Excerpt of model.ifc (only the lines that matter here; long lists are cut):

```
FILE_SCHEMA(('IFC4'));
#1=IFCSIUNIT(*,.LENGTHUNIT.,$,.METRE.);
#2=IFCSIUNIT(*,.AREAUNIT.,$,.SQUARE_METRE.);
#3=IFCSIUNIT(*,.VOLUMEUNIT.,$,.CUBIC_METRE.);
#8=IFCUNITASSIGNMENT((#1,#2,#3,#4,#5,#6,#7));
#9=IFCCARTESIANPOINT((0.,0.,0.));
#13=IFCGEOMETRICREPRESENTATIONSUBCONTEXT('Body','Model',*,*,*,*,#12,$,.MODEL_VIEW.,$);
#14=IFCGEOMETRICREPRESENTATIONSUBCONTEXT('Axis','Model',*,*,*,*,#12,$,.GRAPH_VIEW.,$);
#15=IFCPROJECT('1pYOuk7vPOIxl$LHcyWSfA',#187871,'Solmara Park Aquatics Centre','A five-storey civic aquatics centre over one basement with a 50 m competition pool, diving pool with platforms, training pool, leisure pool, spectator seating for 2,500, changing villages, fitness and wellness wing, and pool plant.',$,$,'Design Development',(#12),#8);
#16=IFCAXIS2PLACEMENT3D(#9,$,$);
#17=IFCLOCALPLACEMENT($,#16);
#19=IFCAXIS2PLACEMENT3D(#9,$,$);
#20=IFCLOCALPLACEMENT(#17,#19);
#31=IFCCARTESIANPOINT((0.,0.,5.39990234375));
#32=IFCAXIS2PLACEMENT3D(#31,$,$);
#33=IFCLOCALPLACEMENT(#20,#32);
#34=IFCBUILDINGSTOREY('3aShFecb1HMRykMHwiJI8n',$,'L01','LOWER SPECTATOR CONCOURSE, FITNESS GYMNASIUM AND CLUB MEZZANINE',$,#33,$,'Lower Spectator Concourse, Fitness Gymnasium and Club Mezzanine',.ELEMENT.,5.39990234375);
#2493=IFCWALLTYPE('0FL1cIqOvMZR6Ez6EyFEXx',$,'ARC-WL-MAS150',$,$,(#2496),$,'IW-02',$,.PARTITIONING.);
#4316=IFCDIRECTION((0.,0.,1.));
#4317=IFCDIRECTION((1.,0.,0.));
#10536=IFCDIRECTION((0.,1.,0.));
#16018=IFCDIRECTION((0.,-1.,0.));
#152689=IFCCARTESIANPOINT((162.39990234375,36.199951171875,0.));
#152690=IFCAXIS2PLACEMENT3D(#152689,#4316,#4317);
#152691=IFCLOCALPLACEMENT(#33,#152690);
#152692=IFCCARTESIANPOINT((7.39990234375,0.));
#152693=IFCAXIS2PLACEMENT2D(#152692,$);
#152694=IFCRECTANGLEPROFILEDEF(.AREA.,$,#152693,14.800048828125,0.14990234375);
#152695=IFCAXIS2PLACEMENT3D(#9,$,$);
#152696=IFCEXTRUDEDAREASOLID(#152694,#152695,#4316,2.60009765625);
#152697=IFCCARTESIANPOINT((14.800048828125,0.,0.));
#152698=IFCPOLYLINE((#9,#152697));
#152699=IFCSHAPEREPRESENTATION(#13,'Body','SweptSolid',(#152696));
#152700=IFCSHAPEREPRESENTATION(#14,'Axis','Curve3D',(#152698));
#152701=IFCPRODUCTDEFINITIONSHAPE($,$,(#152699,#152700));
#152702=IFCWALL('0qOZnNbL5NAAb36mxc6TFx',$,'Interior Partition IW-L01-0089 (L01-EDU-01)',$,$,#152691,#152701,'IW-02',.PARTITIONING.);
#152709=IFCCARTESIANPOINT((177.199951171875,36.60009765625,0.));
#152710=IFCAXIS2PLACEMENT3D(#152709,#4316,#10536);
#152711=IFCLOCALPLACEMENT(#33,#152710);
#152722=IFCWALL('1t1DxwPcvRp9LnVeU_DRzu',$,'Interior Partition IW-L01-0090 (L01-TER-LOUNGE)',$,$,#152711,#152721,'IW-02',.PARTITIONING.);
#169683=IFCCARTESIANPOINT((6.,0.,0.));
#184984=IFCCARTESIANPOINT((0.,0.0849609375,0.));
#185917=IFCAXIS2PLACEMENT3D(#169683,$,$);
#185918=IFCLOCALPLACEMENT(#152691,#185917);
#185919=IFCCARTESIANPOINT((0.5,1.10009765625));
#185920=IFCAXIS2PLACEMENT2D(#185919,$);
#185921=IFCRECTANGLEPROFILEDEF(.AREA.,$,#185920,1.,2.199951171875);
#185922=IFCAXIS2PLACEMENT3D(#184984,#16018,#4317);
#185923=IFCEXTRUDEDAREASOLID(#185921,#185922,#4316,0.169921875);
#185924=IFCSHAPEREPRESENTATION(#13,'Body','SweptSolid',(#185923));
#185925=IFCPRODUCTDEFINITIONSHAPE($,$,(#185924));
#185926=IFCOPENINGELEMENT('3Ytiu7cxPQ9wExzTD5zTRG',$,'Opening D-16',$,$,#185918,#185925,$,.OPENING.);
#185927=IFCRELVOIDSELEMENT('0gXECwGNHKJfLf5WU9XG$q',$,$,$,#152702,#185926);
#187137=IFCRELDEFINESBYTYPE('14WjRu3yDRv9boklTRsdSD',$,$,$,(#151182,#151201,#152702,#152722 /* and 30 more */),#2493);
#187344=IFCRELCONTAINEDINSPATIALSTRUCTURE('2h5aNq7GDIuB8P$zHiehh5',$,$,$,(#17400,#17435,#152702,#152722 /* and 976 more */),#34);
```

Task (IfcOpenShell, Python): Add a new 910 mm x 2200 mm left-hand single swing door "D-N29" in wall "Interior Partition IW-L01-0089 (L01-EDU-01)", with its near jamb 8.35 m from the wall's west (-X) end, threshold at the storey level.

```python
import numpy as np
import ifcopenshell
import ifcopenshell.api.feature
import ifcopenshell.api.geometry
import ifcopenshell.api.root
import ifcopenshell.api.spatial
import ifcopenshell.geom
import ifcopenshell.util.element
import ifcopenshell.util.placement
import ifcopenshell.util.representation
import ifcopenshell.util.shape
import ifcopenshell.util.unit

model = ifcopenshell.open("model.ifc")
unit_scale = ifcopenshell.util.unit.calculate_unit_scale(model)
settings = ifcopenshell.geom.settings()


def volume(element):
    """Net volume in cubic metres, openings subtracted."""
    shape = ifcopenshell.geom.create_shape(settings, element)
    return ifcopenshell.util.shape.get_volume(shape.geometry)


wall = model.by_guid("0qOZnNbL5NAAb36mxc6TFx")
storey = ifcopenshell.util.element.get_container(wall, ifc_class="IfcBuildingStorey")
context = ifcopenshell.util.representation.get_context(model, "Model", "Body", "MODEL_VIEW")
before = volume(wall)

width, height, from_end, sill = 0.91, 2.2, 8.35, 0.0  # metres

# The wall runs along its own X axis, and the end named is its -X end.
wall_shape = ifcopenshell.geom.create_shape(settings, wall)
x, y, z = ifcopenshell.util.shape.get_vertices(wall_shape.geometry).T
start = x.min() + from_end
face, thickness = float(y.min()), float(y.max() - y.min())
wall_matrix = ifcopenshell.util.placement.get_local_placement(wall.ObjectPlacement)
level = ifcopenshell.util.placement.get_local_placement(storey.ObjectPlacement)[2, 3]


def in_wall(x, y):
    """Placement at x, y metres in the wall's axes, at sill height."""
    matrix = wall_matrix.copy()
    matrix[:, 3] = wall_matrix @ np.array([x / unit_scale, y / unit_scale, 0.0, 1.0])
    matrix[2, 3] = level + sill / unit_scale
    return matrix


# Opening: a box that overshoots both wall faces by 50 mm.
opening = ifcopenshell.api.root.create_entity(model, ifc_class="IfcOpeningElement", predefined_type="OPENING")
box = ifcopenshell.api.geometry.add_wall_representation(
    model, context=context, length=width, height=height, thickness=thickness + 0.1
)
ifcopenshell.api.geometry.assign_representation(model, product=opening, representation=box)
ifcopenshell.api.geometry.edit_object_placement(model, product=opening, matrix=in_wall(start, face - 0.05), is_si=False)
ifcopenshell.api.feature.add_feature(model, feature=opening, element=wall)

door = ifcopenshell.api.root.create_entity(model, ifc_class="IfcDoor", name="D-N29", predefined_type="DOOR")
door.OverallWidth, door.OverallHeight = width / unit_scale, height / unit_scale
door.OperationType = "SINGLE_SWING_LEFT"
body = ifcopenshell.api.geometry.add_door_representation(
    model,
    context=context,
    overall_width=door.OverallWidth,
    overall_height=door.OverallHeight,
    operation_type="SINGLE_SWING_LEFT",
    lining_properties={"LiningDepth": thickness / unit_scale, "ThresholdDepth": thickness / unit_scale},
)
ifcopenshell.api.geometry.assign_representation(model, product=door, representation=body)
ifcopenshell.api.spatial.assign_container(model, products=[door], relating_structure=storey)
ifcopenshell.api.feature.add_filling(model, opening=opening, element=door)

# The lining spans the wall, so the door starts at the wall face.
ifcopenshell.api.geometry.edit_object_placement(model, product=door, matrix=in_wall(start, face), is_si=False)

after = volume(wall)

print(f"wall volume {before:.3f} -> {after:.3f} m3")

model.write("model_v2.ifc")
```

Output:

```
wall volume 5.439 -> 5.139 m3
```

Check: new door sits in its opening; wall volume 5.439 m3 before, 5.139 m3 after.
